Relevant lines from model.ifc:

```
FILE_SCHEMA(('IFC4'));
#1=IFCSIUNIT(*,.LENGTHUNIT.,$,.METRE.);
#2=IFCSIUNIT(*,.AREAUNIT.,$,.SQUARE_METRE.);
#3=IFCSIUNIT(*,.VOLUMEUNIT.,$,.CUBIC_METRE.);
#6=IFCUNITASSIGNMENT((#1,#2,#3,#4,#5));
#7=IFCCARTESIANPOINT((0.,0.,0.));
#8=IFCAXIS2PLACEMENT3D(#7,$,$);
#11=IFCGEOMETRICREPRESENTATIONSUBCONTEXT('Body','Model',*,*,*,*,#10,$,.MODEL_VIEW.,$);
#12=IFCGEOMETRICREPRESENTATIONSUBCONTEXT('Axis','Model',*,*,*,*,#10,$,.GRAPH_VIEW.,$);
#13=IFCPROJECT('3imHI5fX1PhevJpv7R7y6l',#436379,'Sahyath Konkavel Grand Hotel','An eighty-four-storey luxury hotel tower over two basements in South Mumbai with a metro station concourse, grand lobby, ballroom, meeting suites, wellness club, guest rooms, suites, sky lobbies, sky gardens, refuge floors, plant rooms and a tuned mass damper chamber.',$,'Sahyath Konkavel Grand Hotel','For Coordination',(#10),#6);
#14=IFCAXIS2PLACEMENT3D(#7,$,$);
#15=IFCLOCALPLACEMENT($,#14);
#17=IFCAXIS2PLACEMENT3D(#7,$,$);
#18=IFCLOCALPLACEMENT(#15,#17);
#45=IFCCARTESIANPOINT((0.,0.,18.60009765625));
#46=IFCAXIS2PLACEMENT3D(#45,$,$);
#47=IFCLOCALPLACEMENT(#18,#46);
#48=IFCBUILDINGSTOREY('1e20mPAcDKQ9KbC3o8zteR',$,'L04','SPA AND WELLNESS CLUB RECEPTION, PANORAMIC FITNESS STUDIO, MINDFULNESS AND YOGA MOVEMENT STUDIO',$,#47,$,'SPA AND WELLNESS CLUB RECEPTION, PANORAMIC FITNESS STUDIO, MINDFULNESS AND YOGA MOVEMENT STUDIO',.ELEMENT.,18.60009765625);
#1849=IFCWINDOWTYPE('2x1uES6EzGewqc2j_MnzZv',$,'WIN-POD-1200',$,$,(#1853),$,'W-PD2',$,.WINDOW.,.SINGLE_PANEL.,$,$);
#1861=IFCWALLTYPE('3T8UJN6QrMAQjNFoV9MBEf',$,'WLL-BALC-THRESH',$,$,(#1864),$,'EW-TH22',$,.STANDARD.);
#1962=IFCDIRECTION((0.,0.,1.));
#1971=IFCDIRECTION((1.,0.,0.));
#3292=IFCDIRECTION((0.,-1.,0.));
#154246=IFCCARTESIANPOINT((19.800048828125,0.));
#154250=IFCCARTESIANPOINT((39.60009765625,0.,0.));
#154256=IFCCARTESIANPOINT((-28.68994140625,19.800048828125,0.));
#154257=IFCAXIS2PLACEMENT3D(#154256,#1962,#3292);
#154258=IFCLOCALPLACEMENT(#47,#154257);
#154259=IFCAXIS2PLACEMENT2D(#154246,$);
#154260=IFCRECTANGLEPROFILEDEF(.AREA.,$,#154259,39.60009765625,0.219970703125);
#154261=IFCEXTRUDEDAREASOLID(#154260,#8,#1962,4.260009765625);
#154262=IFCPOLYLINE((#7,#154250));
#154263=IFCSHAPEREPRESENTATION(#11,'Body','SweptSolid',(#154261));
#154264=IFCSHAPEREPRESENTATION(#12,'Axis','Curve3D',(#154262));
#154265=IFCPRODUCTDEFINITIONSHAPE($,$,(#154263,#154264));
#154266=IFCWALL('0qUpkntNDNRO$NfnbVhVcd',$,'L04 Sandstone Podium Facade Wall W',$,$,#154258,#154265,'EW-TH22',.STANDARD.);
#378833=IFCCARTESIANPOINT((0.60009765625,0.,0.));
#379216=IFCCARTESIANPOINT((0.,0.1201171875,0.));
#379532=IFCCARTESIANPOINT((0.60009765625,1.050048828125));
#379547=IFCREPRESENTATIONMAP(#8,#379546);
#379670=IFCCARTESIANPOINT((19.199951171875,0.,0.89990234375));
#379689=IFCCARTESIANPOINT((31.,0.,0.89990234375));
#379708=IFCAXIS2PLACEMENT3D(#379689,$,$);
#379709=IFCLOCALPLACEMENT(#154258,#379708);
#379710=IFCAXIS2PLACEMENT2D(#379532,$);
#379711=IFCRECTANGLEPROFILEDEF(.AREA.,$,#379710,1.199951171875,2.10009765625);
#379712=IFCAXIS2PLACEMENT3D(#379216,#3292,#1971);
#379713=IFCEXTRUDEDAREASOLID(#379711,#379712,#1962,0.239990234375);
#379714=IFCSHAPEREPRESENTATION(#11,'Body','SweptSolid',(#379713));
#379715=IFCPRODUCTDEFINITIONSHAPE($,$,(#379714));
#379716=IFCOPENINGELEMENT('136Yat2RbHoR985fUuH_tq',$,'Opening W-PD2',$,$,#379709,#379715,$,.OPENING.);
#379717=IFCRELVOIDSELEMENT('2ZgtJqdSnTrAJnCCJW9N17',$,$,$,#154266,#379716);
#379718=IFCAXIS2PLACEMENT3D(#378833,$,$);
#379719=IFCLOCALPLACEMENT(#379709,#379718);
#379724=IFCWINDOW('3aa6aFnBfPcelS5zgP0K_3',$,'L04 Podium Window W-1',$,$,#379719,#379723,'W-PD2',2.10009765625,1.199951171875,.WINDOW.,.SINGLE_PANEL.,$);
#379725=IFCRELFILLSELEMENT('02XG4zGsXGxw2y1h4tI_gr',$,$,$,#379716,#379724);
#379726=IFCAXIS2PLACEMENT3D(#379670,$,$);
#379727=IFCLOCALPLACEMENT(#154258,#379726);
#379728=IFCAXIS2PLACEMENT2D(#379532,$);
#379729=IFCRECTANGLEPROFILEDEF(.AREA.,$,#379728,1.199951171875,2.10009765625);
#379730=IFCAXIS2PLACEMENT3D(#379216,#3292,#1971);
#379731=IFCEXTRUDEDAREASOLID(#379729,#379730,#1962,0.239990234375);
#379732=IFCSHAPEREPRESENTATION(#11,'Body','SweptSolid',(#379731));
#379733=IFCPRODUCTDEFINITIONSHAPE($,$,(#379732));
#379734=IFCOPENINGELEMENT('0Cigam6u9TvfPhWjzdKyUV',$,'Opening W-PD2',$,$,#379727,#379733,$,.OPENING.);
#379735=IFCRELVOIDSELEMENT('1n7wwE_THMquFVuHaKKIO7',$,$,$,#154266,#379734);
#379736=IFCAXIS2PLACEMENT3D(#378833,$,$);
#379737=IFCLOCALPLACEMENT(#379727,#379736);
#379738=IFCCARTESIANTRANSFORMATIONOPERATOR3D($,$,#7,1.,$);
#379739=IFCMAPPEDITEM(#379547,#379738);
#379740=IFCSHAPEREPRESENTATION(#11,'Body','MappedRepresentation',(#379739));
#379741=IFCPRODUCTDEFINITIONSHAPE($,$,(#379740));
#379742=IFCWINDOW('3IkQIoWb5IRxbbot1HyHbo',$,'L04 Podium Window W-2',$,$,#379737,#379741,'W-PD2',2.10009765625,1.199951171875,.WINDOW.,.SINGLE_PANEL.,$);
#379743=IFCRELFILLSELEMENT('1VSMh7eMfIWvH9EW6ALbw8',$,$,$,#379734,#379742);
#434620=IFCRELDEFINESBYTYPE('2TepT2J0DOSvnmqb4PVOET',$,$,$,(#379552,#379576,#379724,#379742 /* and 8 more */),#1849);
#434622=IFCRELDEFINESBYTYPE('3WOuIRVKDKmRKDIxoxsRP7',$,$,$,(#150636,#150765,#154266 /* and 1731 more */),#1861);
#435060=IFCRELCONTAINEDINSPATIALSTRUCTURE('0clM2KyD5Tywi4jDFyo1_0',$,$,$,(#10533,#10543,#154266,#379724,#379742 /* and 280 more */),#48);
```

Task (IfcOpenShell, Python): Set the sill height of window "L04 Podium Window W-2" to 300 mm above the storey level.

```python
import numpy as np
import ifcopenshell
import ifcopenshell.api.geometry
import ifcopenshell.geom
import ifcopenshell.util.element
import ifcopenshell.util.placement
import ifcopenshell.util.shape
import ifcopenshell.util.unit

model = ifcopenshell.open("model.ifc")
unit_scale = ifcopenshell.util.unit.calculate_unit_scale(model)

window = model.by_guid("3IkQIoWb5IRxbbot1HyHbo")
opening = window.FillsVoids[0].RelatingOpeningElement
storey = ifcopenshell.util.element.get_container(window, ifc_class="IfcBuildingStorey")
level = ifcopenshell.util.placement.get_local_placement(storey.ObjectPlacement)[2, 3]

# The opening's origin need not be at the sill, so measure its lowest point.
shape = ifcopenshell.geom.create_shape(ifcopenshell.geom.settings(), opening)
bottom = ifcopenshell.util.shape.get_shape_bottom_elevation(shape, shape.geometry) / unit_scale
dz = level + 0.3 / unit_scale - bottom

shift = np.array([0.0, 0.0, dz])
# The window is placed relative to its opening, so it follows when the opening moves.
matrix = ifcopenshell.util.placement.get_local_placement(opening.ObjectPlacement)
matrix[:3, 3] += shift
ifcopenshell.api.geometry.edit_object_placement(
    model, product=opening, matrix=matrix, is_si=False, should_transform_children=True
)

print(f"moved by {dz * unit_scale:+.3f} m")

model.write("model_v2.ifc")
```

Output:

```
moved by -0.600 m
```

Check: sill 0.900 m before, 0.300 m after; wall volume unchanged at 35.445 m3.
